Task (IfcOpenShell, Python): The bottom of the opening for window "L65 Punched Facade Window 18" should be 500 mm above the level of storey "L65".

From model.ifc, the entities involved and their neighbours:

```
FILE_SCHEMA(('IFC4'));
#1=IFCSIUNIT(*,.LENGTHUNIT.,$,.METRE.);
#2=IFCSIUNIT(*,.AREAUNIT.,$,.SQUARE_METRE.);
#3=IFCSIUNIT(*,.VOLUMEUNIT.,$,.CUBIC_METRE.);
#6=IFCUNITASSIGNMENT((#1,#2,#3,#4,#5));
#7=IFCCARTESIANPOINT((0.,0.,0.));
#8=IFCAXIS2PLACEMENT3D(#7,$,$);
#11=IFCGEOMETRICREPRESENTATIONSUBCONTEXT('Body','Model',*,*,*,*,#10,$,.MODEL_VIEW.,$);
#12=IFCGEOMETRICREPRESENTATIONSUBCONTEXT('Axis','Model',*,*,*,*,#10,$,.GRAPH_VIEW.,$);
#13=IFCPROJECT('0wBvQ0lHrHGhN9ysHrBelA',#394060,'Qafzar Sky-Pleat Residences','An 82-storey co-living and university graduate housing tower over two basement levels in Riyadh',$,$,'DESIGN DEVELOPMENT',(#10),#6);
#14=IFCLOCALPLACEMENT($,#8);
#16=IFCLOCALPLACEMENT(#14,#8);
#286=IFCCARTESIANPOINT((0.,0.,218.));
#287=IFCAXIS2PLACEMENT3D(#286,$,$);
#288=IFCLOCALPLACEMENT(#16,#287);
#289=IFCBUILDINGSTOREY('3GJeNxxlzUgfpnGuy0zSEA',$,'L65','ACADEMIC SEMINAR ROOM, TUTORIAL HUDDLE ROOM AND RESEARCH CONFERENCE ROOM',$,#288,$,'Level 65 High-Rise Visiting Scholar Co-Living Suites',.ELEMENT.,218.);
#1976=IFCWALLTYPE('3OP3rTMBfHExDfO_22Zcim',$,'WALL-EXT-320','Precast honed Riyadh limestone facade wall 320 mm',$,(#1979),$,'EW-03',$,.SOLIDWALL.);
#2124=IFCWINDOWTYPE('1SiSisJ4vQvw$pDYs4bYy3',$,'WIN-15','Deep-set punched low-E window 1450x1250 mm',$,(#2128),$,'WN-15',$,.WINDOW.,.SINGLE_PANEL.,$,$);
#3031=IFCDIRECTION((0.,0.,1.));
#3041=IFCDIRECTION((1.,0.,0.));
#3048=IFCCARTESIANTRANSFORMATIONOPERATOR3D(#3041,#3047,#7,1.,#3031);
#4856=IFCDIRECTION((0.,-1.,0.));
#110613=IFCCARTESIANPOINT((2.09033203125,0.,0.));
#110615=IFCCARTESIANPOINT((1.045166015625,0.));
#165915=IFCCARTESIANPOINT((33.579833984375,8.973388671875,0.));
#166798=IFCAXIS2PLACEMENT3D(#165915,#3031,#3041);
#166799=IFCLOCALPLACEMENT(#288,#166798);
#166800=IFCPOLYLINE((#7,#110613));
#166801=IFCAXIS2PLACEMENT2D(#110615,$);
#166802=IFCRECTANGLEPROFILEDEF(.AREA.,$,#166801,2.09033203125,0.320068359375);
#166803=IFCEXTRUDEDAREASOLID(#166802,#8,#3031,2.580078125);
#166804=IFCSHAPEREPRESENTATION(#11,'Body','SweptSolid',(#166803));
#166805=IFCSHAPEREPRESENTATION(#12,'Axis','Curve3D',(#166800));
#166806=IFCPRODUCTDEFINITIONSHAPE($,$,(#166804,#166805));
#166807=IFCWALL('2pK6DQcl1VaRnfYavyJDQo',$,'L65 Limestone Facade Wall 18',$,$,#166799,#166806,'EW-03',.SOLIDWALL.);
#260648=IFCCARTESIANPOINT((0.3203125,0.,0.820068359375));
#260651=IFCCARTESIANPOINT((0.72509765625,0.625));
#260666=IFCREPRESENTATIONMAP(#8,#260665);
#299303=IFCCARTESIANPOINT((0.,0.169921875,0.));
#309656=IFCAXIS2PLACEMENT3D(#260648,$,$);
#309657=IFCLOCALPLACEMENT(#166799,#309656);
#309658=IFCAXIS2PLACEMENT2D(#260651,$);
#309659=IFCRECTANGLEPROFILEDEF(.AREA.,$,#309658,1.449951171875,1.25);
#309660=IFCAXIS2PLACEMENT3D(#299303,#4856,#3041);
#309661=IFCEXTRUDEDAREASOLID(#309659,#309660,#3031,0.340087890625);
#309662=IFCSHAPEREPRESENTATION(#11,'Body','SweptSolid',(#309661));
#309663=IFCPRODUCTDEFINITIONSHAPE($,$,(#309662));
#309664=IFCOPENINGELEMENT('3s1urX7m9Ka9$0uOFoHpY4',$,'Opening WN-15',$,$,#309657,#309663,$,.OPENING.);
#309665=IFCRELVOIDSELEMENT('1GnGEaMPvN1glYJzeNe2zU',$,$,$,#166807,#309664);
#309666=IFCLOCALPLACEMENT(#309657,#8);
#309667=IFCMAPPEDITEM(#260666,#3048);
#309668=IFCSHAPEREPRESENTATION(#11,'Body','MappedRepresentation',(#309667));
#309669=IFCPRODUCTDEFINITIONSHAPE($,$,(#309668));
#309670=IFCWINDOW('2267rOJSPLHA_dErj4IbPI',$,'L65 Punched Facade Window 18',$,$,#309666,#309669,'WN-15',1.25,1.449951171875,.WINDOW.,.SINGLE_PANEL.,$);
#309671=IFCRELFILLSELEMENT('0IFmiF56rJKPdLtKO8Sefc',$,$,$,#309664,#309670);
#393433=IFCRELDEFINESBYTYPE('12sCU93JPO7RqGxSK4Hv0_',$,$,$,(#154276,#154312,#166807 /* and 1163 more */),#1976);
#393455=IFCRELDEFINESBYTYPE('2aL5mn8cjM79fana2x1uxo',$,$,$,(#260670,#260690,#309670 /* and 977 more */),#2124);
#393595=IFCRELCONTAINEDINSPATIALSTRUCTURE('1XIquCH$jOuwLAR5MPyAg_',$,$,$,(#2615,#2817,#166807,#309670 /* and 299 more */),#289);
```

```python
import numpy as np
import ifcopenshell
import ifcopenshell.api.geometry
import ifcopenshell.geom
import ifcopenshell.util.element
import ifcopenshell.util.placement
import ifcopenshell.util.shape
import ifcopenshell.util.unit

model = ifcopenshell.open("model.ifc")
unit_scale = ifcopenshell.util.unit.calculate_unit_scale(model)

window = model.by_guid("2267rOJSPLHA_dErj4IbPI")
opening = window.FillsVoids[0].RelatingOpeningElement
storey = ifcopenshell.util.element.get_container(window, ifc_class="IfcBuildingStorey")
level = ifcopenshell.util.placement.get_local_placement(storey.ObjectPlacement)[2, 3]

# The opening's origin need not be at the sill, so measure its lowest point.
shape = ifcopenshell.geom.create_shape(ifcopenshell.geom.settings(), opening)
bottom = ifcopenshell.util.shape.get_shape_bottom_elevation(shape, shape.geometry) / unit_scale
dz = level + 0.5 - bottom

shift = np.array([0.0, 0.0, dz])
# The window is placed relative to its opening, so it follows when the opening moves.
matrix = ifcopenshell.util.placement.get_local_placement(opening.ObjectPlacement)
matrix[:3, 3] += shift
ifcopenshell.api.geometry.edit_object_placement(
    model, product=opening, matrix=matrix, is_si=False, should_transform_children=True
)

print(f"moved by {dz * unit_scale:+.3f} m")

model.write("model_rev.ifc")
```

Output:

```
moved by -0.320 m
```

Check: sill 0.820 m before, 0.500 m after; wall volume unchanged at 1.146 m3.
